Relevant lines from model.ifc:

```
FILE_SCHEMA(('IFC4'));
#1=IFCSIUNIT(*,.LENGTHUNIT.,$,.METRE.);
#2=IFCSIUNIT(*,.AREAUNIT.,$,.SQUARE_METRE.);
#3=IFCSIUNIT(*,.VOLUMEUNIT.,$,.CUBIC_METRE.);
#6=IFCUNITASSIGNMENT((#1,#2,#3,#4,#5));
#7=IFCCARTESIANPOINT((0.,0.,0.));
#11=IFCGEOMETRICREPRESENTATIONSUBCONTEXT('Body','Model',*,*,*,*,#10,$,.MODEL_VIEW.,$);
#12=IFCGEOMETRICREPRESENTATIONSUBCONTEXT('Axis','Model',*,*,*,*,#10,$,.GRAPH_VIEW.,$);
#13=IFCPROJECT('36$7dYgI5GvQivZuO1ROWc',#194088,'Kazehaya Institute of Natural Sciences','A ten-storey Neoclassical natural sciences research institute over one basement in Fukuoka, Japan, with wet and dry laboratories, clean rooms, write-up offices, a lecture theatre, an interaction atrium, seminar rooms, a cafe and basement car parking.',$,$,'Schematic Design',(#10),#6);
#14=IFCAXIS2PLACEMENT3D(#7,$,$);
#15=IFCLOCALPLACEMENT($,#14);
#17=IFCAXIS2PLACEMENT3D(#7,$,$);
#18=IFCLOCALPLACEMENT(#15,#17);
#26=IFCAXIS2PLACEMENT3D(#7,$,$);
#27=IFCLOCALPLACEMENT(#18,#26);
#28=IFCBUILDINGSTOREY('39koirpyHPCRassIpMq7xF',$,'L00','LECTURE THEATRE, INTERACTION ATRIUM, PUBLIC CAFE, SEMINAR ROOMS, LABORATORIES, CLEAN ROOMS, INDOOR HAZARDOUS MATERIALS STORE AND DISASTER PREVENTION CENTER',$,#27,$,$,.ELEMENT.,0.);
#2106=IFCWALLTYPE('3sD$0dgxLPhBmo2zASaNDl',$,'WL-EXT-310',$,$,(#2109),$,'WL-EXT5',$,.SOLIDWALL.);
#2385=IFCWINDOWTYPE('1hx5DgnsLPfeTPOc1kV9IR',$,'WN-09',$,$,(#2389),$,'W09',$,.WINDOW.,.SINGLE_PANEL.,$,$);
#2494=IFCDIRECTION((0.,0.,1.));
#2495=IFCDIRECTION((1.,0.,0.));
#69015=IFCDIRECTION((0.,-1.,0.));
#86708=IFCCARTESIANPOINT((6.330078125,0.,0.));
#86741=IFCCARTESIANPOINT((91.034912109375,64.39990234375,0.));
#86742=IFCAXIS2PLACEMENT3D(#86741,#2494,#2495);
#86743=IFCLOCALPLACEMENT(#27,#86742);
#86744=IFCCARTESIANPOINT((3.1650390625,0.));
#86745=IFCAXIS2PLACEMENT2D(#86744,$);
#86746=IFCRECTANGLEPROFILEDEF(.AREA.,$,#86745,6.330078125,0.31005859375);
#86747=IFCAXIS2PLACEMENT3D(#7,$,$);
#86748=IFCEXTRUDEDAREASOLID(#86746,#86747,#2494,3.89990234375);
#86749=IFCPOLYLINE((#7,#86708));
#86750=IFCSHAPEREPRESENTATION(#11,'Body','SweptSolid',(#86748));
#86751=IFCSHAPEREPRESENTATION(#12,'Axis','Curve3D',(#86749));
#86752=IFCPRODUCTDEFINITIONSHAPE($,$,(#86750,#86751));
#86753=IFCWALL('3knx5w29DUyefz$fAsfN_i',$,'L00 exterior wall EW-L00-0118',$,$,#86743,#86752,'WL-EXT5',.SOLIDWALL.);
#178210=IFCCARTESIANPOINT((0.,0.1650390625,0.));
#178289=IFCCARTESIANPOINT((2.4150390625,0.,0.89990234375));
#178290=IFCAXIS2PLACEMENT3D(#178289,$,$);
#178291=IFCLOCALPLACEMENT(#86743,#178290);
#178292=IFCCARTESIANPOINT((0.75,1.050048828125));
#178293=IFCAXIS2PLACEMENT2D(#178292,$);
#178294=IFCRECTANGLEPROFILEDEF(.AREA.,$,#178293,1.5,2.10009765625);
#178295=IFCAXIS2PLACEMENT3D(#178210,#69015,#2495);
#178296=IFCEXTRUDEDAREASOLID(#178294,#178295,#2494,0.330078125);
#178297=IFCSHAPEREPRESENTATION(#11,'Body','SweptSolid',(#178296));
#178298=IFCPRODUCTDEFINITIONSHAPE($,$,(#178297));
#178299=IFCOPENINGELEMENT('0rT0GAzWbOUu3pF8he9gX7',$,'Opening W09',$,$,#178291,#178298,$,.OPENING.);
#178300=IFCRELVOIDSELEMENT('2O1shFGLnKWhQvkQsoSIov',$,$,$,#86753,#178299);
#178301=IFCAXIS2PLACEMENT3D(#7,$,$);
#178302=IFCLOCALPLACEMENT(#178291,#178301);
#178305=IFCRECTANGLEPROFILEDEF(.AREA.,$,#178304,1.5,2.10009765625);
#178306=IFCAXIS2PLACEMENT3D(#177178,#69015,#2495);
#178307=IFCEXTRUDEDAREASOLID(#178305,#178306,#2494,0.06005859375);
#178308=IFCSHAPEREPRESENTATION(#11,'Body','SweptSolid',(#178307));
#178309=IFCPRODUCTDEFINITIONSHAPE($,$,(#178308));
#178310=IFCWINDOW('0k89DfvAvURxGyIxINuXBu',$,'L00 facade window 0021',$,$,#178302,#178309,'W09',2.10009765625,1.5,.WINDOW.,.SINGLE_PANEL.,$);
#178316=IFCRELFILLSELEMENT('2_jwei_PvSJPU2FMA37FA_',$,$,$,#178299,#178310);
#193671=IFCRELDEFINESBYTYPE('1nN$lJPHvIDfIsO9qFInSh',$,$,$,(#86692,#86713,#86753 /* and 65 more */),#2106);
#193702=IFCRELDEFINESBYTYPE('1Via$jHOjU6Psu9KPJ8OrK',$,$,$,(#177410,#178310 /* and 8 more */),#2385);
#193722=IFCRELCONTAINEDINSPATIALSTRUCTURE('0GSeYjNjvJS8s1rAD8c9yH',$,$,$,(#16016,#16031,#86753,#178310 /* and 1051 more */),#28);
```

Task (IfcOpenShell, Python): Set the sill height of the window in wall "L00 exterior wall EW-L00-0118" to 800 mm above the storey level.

```python
import numpy as np
import ifcopenshell
import ifcopenshell.api.geometry
import ifcopenshell.geom
import ifcopenshell.util.element
import ifcopenshell.util.placement
import ifcopenshell.util.shape
import ifcopenshell.util.unit

model = ifcopenshell.open("model.ifc")
unit_scale = ifcopenshell.util.unit.calculate_unit_scale(model)

window = model.by_guid("0k89DfvAvURxGyIxINuXBu")
opening = window.FillsVoids[0].RelatingOpeningElement
storey = ifcopenshell.util.element.get_container(window, ifc_class="IfcBuildingStorey")
level = ifcopenshell.util.placement.get_local_placement(storey.ObjectPlacement)[2, 3]

# The opening's origin need not be at the sill, so measure its lowest point.
shape = ifcopenshell.geom.create_shape(ifcopenshell.geom.settings(), opening)
bottom = ifcopenshell.util.shape.get_shape_bottom_elevation(shape, shape.geometry) / unit_scale
dz = level + 0.8 / unit_scale - bottom

shift = np.array([0.0, 0.0, dz])
# The window is placed relative to its opening, so it follows when the opening moves.
matrix = ifcopenshell.util.placement.get_local_placement(opening.ObjectPlacement)
matrix[:3, 3] += shift
ifcopenshell.api.geometry.edit_object_placement(
    model, product=opening, matrix=matrix, is_si=False, should_transform_children=True
)

print(f"moved by {dz * unit_scale:+.3f} m")

model.write("model_edited.ifc")
```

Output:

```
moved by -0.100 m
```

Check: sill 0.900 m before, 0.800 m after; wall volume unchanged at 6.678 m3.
